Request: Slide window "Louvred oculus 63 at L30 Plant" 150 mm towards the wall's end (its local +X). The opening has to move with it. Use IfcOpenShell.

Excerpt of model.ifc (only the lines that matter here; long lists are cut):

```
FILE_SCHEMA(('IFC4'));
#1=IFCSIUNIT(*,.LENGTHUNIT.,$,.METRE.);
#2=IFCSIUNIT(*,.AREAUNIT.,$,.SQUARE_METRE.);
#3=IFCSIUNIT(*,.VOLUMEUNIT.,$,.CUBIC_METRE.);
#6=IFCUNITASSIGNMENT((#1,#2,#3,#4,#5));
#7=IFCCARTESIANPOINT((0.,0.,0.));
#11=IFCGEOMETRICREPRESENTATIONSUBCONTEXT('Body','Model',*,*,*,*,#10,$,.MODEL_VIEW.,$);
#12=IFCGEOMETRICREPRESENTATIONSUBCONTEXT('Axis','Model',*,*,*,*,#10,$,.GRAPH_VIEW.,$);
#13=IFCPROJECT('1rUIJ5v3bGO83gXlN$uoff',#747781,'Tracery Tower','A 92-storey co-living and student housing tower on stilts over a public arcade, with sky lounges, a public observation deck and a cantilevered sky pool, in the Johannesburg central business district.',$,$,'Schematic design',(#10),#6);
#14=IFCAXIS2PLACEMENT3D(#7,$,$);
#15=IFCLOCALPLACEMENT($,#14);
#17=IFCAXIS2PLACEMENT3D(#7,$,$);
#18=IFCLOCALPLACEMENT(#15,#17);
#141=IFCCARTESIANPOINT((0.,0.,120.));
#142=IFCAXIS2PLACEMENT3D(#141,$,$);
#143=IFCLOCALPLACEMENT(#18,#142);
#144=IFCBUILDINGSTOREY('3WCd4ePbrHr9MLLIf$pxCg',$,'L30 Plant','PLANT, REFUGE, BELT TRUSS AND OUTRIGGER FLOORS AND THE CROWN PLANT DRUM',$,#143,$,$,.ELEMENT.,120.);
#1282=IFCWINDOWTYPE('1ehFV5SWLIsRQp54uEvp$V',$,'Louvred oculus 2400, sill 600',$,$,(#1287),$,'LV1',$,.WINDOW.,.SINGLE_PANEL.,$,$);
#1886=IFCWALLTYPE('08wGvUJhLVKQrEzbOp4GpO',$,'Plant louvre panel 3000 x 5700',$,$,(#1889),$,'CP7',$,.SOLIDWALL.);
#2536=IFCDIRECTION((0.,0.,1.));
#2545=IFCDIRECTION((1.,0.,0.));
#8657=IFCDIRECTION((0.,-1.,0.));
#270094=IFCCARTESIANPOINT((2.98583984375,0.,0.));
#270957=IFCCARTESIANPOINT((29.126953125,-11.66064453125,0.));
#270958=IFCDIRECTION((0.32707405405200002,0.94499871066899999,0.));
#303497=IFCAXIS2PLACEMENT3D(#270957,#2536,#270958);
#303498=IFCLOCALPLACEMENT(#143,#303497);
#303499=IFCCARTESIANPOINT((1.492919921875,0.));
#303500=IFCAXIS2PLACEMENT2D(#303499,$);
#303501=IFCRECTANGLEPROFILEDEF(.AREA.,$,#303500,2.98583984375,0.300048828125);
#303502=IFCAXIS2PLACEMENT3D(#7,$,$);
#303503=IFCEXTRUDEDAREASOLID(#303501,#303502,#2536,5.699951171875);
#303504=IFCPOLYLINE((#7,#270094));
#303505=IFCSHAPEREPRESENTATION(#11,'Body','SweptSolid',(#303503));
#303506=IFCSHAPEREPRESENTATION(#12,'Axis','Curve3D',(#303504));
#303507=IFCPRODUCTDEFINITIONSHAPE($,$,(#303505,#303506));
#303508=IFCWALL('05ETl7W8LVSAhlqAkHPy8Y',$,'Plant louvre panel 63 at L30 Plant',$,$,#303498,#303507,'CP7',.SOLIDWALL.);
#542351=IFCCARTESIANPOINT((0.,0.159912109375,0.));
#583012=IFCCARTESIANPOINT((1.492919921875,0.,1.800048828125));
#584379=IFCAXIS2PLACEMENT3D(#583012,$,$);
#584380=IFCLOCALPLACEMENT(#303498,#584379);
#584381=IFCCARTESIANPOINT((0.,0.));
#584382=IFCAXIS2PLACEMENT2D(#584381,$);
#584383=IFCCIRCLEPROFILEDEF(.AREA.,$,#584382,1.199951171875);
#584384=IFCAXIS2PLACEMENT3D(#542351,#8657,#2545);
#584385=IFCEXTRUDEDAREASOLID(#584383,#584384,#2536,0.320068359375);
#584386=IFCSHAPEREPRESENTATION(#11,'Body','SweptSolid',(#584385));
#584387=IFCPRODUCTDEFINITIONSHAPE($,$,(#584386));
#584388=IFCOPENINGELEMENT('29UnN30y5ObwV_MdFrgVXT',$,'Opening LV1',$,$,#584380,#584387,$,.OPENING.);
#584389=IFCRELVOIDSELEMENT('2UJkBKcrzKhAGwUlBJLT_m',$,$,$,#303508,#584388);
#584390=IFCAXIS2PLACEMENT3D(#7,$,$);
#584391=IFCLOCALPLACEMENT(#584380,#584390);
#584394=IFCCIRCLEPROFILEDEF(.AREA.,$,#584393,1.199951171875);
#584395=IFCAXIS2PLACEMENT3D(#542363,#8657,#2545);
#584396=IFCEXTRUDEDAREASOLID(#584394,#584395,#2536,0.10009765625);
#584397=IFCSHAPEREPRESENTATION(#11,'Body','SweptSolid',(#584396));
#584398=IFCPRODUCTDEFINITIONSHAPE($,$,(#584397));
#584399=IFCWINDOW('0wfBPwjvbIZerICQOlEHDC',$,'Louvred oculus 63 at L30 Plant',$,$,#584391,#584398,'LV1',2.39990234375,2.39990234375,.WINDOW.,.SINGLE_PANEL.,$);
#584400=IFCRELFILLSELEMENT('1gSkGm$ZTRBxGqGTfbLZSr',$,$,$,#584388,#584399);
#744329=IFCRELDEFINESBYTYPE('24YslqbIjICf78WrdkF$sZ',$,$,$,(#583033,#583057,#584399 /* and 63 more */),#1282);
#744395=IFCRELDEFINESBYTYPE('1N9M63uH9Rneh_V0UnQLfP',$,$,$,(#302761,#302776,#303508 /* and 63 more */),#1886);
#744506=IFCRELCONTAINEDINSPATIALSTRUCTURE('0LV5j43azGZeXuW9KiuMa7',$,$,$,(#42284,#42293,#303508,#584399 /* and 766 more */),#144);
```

```python
import ifcopenshell
import ifcopenshell.api.geometry
import ifcopenshell.util.placement
import ifcopenshell.util.unit

model = ifcopenshell.open("model.ifc")
unit_scale = ifcopenshell.util.unit.calculate_unit_scale(model)

window = model.by_guid("0wfBPwjvbIZerICQOlEHDC")
opening = window.FillsVoids[0].RelatingOpeningElement
wall = opening.VoidsElements[0].RelatingBuildingElement

wall_matrix = ifcopenshell.util.placement.get_local_placement(wall.ObjectPlacement)
shift = wall_matrix[:3, 0] * 0.15 / unit_scale
before = ifcopenshell.util.placement.get_local_placement(window.ObjectPlacement)[:3, 3].copy()

# The window is placed relative to its opening, so it follows when the opening moves.
matrix = ifcopenshell.util.placement.get_local_placement(opening.ObjectPlacement)
matrix[:3, 3] += shift
ifcopenshell.api.geometry.edit_object_placement(
    model, product=opening, matrix=matrix, is_si=False, should_transform_children=True
)

after = ifcopenshell.util.placement.get_local_placement(window.ObjectPlacement)[:3, 3]
print("window moved by", (after - before).round(3) + 0.0)

model.write("model_v2.ifc")
```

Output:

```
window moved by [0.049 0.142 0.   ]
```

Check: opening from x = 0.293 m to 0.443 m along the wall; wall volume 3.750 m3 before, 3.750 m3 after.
